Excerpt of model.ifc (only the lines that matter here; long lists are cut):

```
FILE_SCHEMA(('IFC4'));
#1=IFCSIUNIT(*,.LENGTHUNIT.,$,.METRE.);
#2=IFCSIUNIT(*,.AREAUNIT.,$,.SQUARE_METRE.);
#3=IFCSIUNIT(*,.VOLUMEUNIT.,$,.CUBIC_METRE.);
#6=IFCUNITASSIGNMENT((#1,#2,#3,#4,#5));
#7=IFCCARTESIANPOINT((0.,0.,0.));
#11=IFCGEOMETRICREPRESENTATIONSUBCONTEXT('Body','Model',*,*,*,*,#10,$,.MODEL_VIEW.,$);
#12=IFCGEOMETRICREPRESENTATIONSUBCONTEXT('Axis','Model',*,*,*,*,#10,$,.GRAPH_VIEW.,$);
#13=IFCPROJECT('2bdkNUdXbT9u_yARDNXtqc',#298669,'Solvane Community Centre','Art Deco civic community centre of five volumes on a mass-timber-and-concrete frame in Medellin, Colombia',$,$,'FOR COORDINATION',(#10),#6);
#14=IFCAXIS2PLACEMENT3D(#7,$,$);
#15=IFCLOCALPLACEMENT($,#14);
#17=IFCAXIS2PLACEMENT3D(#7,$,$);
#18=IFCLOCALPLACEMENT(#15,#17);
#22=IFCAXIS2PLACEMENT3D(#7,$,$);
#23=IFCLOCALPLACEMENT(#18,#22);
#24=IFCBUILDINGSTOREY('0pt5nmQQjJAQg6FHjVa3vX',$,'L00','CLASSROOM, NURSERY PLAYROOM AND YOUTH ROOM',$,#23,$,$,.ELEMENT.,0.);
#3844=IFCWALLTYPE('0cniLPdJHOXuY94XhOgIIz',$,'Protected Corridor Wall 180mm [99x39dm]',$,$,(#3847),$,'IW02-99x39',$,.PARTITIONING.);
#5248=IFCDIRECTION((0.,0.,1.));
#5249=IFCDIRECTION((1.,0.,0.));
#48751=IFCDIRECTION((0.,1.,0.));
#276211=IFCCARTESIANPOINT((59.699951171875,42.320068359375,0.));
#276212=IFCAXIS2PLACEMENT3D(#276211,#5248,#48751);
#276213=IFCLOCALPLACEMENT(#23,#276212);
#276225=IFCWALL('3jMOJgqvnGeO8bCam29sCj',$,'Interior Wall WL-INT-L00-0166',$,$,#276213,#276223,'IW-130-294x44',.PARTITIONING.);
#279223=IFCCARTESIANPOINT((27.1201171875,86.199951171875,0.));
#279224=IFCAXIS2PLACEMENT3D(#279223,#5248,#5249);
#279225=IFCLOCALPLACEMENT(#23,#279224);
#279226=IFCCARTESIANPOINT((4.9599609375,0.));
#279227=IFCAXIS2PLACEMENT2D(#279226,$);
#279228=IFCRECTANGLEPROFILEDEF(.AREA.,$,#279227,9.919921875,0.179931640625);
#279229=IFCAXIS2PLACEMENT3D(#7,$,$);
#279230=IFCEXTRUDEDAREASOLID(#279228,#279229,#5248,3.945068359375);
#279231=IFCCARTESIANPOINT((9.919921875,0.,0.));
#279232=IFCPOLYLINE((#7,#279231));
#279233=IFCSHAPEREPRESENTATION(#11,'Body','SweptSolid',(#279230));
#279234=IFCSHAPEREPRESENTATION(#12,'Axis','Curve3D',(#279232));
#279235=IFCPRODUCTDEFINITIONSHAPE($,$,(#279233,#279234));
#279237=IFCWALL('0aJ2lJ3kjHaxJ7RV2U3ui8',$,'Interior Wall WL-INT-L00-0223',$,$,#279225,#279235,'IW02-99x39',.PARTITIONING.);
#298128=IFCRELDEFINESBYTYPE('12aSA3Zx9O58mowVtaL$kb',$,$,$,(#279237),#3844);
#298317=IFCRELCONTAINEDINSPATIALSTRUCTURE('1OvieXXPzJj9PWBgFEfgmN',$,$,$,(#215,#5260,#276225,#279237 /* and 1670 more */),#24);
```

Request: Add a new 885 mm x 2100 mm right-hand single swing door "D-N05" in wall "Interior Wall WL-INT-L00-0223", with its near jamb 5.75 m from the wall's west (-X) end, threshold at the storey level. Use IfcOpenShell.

```python
import numpy as np
import ifcopenshell
import ifcopenshell.api.feature
import ifcopenshell.api.geometry
import ifcopenshell.api.root
import ifcopenshell.api.spatial
import ifcopenshell.geom
import ifcopenshell.util.element
import ifcopenshell.util.placement
import ifcopenshell.util.representation
import ifcopenshell.util.shape
import ifcopenshell.util.unit

model = ifcopenshell.open("model.ifc")
unit_scale = ifcopenshell.util.unit.calculate_unit_scale(model)
settings = ifcopenshell.geom.settings()


def volume(element):
    """Net volume in cubic metres, openings subtracted."""
    shape = ifcopenshell.geom.create_shape(settings, element)
    return ifcopenshell.util.shape.get_volume(shape.geometry)


wall = model.by_guid("0aJ2lJ3kjHaxJ7RV2U3ui8")
storey = ifcopenshell.util.element.get_container(wall, ifc_class="IfcBuildingStorey")
context = ifcopenshell.util.representation.get_context(model, "Model", "Body", "MODEL_VIEW")
before = volume(wall)

width, height, from_end, sill = 0.885, 2.1, 5.75, 0.0  # metres

# The wall runs along its own X axis, and the end named is its -X end.
wall_shape = ifcopenshell.geom.create_shape(settings, wall)
x, y, z = ifcopenshell.util.shape.get_vertices(wall_shape.geometry).T
start = x.min() + from_end
face, thickness = float(y.min()), float(y.max() - y.min())
wall_matrix = ifcopenshell.util.placement.get_local_placement(wall.ObjectPlacement)
level = ifcopenshell.util.placement.get_local_placement(storey.ObjectPlacement)[2, 3]


def in_wall(x, y):
    """Placement at x, y metres in the wall's axes, at sill height."""
    matrix = wall_matrix.copy()
    matrix[:, 3] = wall_matrix @ np.array([x / unit_scale, y / unit_scale, 0.0, 1.0])
    matrix[2, 3] = level + sill / unit_scale
    return matrix


# Opening: a box that overshoots both wall faces by 50 mm.
opening = ifcopenshell.api.root.create_entity(model, ifc_class="IfcOpeningElement", predefined_type="OPENING")
box = ifcopenshell.api.geometry.add_wall_representation(
    model, context=context, length=width, height=height, thickness=thickness + 0.1
)
ifcopenshell.api.geometry.assign_representation(model, product=opening, representation=box)
ifcopenshell.api.geometry.edit_object_placement(model, product=opening, matrix=in_wall(start, face - 0.05), is_si=False)
ifcopenshell.api.feature.add_feature(model, feature=opening, element=wall)

door = ifcopenshell.api.root.create_entity(model, ifc_class="IfcDoor", name="D-N05", predefined_type="DOOR")
door.OverallWidth, door.OverallHeight = width / unit_scale, height / unit_scale
door.OperationType = "SINGLE_SWING_RIGHT"
body = ifcopenshell.api.geometry.add_door_representation(
    model,
    context=context,
    overall_width=door.OverallWidth,
    overall_height=door.OverallHeight,
    operation_type="SINGLE_SWING_RIGHT",
    lining_properties={"LiningDepth": thickness / unit_scale, "ThresholdDepth": thickness / unit_scale},
)
ifcopenshell.api.geometry.assign_representation(model, product=door, representation=body)
ifcopenshell.api.spatial.assign_container(model, products=[door], relating_structure=storey)
ifcopenshell.api.feature.add_filling(model, opening=opening, element=door)

# The lining spans the wall, so the door starts at the wall face.
ifcopenshell.api.geometry.edit_object_placement(model, product=door, matrix=in_wall(start, face), is_si=False)

after = volume(wall)

print(f"wall volume {before:.3f} -> {after:.3f} m3")

model.write("model-out.ifc")
```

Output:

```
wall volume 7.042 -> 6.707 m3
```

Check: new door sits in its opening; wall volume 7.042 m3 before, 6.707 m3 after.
